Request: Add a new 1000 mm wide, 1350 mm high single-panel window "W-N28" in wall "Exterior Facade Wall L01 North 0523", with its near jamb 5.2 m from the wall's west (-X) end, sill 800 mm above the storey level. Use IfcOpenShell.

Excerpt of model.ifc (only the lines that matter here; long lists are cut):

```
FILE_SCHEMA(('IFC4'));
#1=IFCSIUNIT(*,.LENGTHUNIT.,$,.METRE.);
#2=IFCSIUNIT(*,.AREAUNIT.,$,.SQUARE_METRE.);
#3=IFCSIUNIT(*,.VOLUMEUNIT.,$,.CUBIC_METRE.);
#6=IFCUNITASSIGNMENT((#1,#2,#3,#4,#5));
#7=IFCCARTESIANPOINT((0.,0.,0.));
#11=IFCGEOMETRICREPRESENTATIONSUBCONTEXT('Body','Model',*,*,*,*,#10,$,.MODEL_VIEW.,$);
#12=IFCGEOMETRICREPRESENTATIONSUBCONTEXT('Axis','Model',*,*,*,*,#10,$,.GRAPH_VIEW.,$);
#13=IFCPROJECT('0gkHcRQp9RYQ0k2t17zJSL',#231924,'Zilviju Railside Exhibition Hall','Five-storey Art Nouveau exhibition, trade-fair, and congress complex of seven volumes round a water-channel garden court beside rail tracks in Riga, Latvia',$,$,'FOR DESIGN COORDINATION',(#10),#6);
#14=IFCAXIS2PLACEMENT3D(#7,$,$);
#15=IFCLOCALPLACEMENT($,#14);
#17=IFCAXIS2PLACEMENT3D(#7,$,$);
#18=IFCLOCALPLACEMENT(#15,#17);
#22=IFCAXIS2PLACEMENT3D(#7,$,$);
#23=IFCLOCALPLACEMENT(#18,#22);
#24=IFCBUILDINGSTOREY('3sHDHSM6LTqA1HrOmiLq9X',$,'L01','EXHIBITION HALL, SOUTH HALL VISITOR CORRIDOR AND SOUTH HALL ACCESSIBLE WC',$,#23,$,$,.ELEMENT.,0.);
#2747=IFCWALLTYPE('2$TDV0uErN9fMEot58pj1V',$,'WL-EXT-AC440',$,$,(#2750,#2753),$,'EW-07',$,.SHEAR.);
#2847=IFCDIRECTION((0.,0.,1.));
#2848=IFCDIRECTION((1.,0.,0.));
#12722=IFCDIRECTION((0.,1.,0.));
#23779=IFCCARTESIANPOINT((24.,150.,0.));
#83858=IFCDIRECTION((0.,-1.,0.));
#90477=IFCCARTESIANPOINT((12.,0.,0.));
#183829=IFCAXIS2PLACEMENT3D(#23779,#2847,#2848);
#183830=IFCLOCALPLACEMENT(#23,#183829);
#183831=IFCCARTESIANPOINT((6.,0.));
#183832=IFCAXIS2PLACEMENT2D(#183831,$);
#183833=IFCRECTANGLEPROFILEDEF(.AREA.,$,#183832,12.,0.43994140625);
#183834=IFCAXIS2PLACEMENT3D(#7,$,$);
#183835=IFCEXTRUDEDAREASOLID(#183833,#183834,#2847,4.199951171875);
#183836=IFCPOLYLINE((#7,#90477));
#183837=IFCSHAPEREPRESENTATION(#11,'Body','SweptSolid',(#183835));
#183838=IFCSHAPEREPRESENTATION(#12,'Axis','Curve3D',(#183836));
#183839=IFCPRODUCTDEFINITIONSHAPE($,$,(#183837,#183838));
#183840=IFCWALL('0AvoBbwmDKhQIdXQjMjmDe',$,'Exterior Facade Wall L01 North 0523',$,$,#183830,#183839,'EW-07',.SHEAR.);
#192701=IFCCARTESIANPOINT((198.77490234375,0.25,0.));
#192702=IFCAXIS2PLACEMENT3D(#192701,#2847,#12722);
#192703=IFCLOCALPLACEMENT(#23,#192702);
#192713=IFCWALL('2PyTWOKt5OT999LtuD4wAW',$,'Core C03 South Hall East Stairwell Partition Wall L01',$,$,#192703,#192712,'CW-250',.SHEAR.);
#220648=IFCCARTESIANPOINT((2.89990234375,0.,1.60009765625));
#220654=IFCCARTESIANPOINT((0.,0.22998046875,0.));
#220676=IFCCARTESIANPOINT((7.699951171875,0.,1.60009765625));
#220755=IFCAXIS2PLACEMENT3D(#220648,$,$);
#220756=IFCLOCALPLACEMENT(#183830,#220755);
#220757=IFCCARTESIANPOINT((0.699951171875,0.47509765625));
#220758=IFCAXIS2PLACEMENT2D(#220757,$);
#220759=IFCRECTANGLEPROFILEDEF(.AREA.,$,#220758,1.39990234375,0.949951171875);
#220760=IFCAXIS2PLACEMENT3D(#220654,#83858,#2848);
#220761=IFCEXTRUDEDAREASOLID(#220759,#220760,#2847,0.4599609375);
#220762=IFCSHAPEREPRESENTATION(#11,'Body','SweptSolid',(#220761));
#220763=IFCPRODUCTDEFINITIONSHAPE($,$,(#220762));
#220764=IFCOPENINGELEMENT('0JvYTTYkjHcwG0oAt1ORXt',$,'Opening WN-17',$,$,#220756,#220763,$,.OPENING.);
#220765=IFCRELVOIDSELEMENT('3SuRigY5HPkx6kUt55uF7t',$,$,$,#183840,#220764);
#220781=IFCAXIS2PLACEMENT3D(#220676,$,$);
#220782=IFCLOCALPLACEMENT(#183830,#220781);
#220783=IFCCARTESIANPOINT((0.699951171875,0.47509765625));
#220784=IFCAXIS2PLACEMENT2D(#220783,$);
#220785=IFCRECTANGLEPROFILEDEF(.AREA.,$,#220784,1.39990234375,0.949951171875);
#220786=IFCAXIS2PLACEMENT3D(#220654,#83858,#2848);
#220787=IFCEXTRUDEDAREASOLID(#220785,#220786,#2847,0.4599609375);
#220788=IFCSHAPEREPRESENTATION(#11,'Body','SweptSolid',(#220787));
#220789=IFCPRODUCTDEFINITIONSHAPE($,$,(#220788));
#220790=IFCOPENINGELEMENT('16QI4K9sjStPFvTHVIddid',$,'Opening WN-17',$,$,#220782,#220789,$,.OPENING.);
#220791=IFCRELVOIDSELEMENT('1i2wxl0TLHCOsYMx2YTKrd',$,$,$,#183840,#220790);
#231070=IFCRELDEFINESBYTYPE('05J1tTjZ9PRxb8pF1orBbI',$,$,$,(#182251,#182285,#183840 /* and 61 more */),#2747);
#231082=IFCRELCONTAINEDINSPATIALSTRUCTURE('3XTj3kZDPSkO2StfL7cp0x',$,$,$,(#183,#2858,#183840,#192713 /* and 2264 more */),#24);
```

```python
import numpy as np
import ifcopenshell
import ifcopenshell.api.feature
import ifcopenshell.api.geometry
import ifcopenshell.api.root
import ifcopenshell.api.spatial
import ifcopenshell.geom
import ifcopenshell.util.element
import ifcopenshell.util.placement
import ifcopenshell.util.representation
import ifcopenshell.util.shape
import ifcopenshell.util.unit

model = ifcopenshell.open("model.ifc")
unit_scale = ifcopenshell.util.unit.calculate_unit_scale(model)
settings = ifcopenshell.geom.settings()


def volume(element):
    """Net volume in cubic metres, openings subtracted."""
    shape = ifcopenshell.geom.create_shape(settings, element)
    return ifcopenshell.util.shape.get_volume(shape.geometry)


wall = model.by_id(183840)
storey = ifcopenshell.util.element.get_container(wall, ifc_class="IfcBuildingStorey")
context = ifcopenshell.util.representation.get_context(model, "Model", "Body", "MODEL_VIEW")
before = volume(wall)

width, height, from_end, sill = 1, 1.35, 5.2, 0.8  # metres

# The wall runs along its own X axis, and the end named is its -X end.
wall_shape = ifcopenshell.geom.create_shape(settings, wall)
x, y, z = ifcopenshell.util.shape.get_vertices(wall_shape.geometry).T
start = x.min() + from_end
face, thickness = float(y.min()), float(y.max() - y.min())
wall_matrix = ifcopenshell.util.placement.get_local_placement(wall.ObjectPlacement)
level = ifcopenshell.util.placement.get_local_placement(storey.ObjectPlacement)[2, 3]


def in_wall(x, y):
    """Placement at x, y metres in the wall's axes, at sill height."""
    matrix = wall_matrix.copy()
    matrix[:, 3] = wall_matrix @ np.array([x / unit_scale, y / unit_scale, 0.0, 1.0])
    matrix[2, 3] = level + sill / unit_scale
    return matrix


# Opening: a box that overshoots both wall faces by 50 mm.
opening = ifcopenshell.api.root.create_entity(model, ifc_class="IfcOpeningElement", predefined_type="OPENING")
box = ifcopenshell.api.geometry.add_wall_representation(
    model, context=context, length=width, height=height, thickness=thickness + 0.1
)
ifcopenshell.api.geometry.assign_representation(model, product=opening, representation=box)
ifcopenshell.api.geometry.edit_object_placement(model, product=opening, matrix=in_wall(start, face - 0.05), is_si=False)
ifcopenshell.api.feature.add_feature(model, feature=opening, element=wall)

window = ifcopenshell.api.root.create_entity(model, ifc_class="IfcWindow", name="W-N28", predefined_type="WINDOW")
window.OverallWidth, window.OverallHeight = width / unit_scale, height / unit_scale
window.PartitioningType = "SINGLE_PANEL"
body = ifcopenshell.api.geometry.add_window_representation(
    model,
    context=context,
    overall_width=window.OverallWidth,
    overall_height=window.OverallHeight,
    partition_type="SINGLE_PANEL",
)
ifcopenshell.api.geometry.assign_representation(model, product=window, representation=body)
ifcopenshell.api.spatial.assign_container(model, products=[window], relating_structure=storey)
ifcopenshell.api.feature.add_filling(model, opening=opening, element=window)

# Centre the window in the wall's thickness.
ifcopenshell.api.geometry.edit_object_placement(model, product=window, matrix=in_wall(start, face), is_si=False)
window_shape = ifcopenshell.geom.create_shape(settings, window)
depth = ifcopenshell.util.shape.get_vertices(window_shape.geometry)[:, 1]
offset = face + thickness / 2 - (depth.min() + depth.max()) / 2
ifcopenshell.api.geometry.edit_object_placement(model, product=window, matrix=in_wall(start, offset), is_si=False)

after = volume(wall)

print(f"wall volume {before:.3f} -> {after:.3f} m3")

model.write("model_updated.ifc")
```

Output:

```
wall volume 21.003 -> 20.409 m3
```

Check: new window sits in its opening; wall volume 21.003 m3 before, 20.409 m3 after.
